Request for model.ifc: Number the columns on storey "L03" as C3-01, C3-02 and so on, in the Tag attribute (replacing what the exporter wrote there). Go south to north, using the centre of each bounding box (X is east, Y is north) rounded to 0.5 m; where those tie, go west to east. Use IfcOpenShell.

First a look at what the model holds.

```python
import ifcopenshell
import ifcopenshell.util.element
import ifcopenshell.util.placement

model = ifcopenshell.open("model.ifc")
print(model.schema)
storey = next(s for s in model.by_type("IfcBuildingStorey") if s.Name == "L03")
columns = [e for e in ifcopenshell.util.element.get_decomposition(storey) if e.is_a("IfcColumn")]
for e in sorted(columns, key=lambda e: e.id()):
    origin = ifcopenshell.util.placement.get_local_placement(e.ObjectPlacement)[:3, 3]
    print(e.id(), e.Tag, e.Name, origin.round(2) + 0.0, sep=" | ")
```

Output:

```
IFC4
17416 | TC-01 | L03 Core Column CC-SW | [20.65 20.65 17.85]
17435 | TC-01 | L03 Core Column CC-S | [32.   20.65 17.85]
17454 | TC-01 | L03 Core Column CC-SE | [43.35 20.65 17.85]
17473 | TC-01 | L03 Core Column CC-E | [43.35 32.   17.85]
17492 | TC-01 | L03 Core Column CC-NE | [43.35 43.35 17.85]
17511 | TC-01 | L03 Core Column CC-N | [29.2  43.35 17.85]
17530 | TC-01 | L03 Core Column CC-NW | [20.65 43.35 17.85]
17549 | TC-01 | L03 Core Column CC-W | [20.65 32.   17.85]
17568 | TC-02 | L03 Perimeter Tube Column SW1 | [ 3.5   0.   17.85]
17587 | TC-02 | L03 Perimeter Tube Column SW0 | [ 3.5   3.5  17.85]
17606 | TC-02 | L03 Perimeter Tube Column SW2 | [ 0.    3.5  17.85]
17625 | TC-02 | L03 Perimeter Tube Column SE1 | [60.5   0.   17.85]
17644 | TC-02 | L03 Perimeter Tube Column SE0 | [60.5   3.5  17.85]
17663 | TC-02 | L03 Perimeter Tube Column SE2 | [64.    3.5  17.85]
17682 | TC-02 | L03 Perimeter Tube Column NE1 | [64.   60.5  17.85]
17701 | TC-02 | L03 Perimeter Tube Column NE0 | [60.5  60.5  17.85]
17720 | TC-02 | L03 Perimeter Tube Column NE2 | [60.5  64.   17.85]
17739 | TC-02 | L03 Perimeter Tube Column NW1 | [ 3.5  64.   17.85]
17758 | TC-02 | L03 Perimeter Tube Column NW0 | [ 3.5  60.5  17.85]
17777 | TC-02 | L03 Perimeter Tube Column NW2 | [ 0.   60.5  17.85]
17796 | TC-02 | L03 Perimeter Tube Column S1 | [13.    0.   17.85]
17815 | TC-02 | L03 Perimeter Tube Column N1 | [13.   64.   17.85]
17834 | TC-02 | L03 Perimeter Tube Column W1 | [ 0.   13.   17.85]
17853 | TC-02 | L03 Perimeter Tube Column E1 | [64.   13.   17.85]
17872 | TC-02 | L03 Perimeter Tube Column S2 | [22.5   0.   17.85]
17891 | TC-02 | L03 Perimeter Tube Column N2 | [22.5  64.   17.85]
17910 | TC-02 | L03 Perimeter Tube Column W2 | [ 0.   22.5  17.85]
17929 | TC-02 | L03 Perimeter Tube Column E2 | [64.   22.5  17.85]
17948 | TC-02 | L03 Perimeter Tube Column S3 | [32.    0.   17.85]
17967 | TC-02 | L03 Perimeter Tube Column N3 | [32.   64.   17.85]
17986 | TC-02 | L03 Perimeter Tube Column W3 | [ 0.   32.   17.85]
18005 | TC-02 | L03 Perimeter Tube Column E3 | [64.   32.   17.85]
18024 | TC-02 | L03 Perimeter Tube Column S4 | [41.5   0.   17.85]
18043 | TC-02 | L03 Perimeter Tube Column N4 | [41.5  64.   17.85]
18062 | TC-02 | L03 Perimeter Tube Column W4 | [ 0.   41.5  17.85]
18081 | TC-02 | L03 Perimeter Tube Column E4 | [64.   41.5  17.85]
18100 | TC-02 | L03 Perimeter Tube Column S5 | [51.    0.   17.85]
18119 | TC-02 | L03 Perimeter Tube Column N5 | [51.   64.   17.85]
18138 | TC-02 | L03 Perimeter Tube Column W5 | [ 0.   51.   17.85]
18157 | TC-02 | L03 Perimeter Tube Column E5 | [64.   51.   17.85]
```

```python
import ifcopenshell
import ifcopenshell.geom
import ifcopenshell.util.element
import ifcopenshell.util.shape

model = ifcopenshell.open("model.ifc")
settings = ifcopenshell.geom.settings()
settings.set("use-world-coords", True)


def centre(element):
    shape = ifcopenshell.geom.create_shape(settings, element)
    return ifcopenshell.util.shape.get_bbox_centroid(shape.geometry)


storey = next(s for s in model.by_type("IfcBuildingStorey") if s.Name == "L03")
columns = [e for e in ifcopenshell.util.element.get_decomposition(storey) if e.is_a("IfcColumn")]

# Insertion points can sit at a corner or the storey origin, so sort by the geometry (in metres).
centres = {e: centre(e) for e in columns}
columns.sort(key=lambda e: (round(centres[e][1] / 0.5), centres[e][0]))

for i, e in enumerate(columns, start=1):
    number = f"C3-{i:02d}"
    e.Tag = number
    print(e.id(), number)

model.write("model_updated.ifc")
```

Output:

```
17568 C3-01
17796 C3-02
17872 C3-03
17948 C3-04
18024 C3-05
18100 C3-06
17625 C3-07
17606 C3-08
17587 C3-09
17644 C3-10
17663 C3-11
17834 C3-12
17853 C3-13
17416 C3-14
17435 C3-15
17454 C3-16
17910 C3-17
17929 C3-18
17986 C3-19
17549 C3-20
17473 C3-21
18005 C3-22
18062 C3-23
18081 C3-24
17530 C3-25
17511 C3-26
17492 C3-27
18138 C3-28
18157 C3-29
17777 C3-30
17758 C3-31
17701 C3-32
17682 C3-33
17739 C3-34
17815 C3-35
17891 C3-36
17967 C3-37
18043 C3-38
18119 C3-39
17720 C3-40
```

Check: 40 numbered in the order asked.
